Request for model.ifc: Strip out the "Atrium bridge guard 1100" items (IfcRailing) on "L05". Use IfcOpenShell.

First a look at what the model holds.

```python
import ifcopenshell
import ifcopenshell.util.element

model = ifcopenshell.open("model.ifc")
print(model.schema)
storey = next(s for s in model.by_type("IfcBuildingStorey") if s.Name == "L05")
railings = [e for e in ifcopenshell.util.element.get_decomposition(storey) if e.is_a("IfcRailing")]
seen = {}
for e in railings:
    element_type = ifcopenshell.util.element.get_type(e)
    name = element_type.Name if element_type not in (None, e) else None
    seen[name] = seen.get(name, 0) + 1
for name, count in sorted(seen.items(), key=str):
    print(count, "x", name)
```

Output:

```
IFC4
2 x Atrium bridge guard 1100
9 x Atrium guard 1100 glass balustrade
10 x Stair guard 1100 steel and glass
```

```python
import ifcopenshell
import ifcopenshell.api.root
import ifcopenshell.util.element

model = ifcopenshell.open("model.ifc")

storey = next(s for s in model.by_type("IfcBuildingStorey") if s.Name == "L05")
railings = [e for e in ifcopenshell.util.element.get_decomposition(storey) if e.is_a("IfcRailing")]
targets = [e for e in railings if (t := ifcopenshell.util.element.get_type(e)) not in (None, e) and t.Name == "Atrium bridge guard 1100"]

for e in targets:
    ifcopenshell.api.root.remove_product(model, product=e)
print(len(targets), "removed")

model.write("model_v2.ifc")
```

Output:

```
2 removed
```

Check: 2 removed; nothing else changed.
